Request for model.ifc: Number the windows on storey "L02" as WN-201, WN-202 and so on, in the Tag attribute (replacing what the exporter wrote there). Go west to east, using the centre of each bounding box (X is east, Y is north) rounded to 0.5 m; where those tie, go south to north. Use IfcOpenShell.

First a look at what the model holds.

```python
import ifcopenshell
import ifcopenshell.util.element
import ifcopenshell.util.placement

model = ifcopenshell.open("model.ifc")
print(model.schema)
storey = next(s for s in model.by_type("IfcBuildingStorey") if s.Name == "L02")
windows = [e for e in ifcopenshell.util.element.get_decomposition(storey) if e.is_a("IfcWindow")]
for e in sorted(windows, key=lambda e: e.id()):
    origin = ifcopenshell.util.placement.get_local_placement(e.ObjectPlacement)[:3, 3]
    print(e.id(), e.Tag, e.Name, origin.round(2) + 0.0, sep=" | ")
```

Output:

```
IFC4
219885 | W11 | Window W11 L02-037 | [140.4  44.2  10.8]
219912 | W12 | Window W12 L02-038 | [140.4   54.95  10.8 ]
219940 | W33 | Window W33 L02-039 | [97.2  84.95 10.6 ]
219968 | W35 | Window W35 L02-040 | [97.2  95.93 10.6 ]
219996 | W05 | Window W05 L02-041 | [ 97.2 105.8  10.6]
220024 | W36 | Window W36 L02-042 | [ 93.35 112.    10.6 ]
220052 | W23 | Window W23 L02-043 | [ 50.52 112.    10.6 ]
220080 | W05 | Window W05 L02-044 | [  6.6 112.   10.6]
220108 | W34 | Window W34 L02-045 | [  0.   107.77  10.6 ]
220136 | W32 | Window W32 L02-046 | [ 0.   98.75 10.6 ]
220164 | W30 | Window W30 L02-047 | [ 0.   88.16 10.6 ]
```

```python
import ifcopenshell
import ifcopenshell.geom
import ifcopenshell.util.element
import ifcopenshell.util.shape

model = ifcopenshell.open("model.ifc")
settings = ifcopenshell.geom.settings()
settings.set("use-world-coords", True)


def centre(element):
    shape = ifcopenshell.geom.create_shape(settings, element)
    return ifcopenshell.util.shape.get_bbox_centroid(shape.geometry)


storey = next(s for s in model.by_type("IfcBuildingStorey") if s.Name == "L02")
windows = [e for e in ifcopenshell.util.element.get_decomposition(storey) if e.is_a("IfcWindow")]

# Insertion points can sit at a corner or the storey origin, so sort by the geometry (in metres).
centres = {e: centre(e) for e in windows}
windows.sort(key=lambda e: (round(centres[e][0] / 0.5), centres[e][1]))

for i, e in enumerate(windows, start=1):
    number = f"WN-2{i:02d}"
    e.Tag = number
    print(e.id(), number)

model.write("model-out.ifc")
```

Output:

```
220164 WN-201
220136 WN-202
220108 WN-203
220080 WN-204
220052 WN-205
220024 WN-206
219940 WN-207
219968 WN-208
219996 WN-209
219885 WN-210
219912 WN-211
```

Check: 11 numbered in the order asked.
